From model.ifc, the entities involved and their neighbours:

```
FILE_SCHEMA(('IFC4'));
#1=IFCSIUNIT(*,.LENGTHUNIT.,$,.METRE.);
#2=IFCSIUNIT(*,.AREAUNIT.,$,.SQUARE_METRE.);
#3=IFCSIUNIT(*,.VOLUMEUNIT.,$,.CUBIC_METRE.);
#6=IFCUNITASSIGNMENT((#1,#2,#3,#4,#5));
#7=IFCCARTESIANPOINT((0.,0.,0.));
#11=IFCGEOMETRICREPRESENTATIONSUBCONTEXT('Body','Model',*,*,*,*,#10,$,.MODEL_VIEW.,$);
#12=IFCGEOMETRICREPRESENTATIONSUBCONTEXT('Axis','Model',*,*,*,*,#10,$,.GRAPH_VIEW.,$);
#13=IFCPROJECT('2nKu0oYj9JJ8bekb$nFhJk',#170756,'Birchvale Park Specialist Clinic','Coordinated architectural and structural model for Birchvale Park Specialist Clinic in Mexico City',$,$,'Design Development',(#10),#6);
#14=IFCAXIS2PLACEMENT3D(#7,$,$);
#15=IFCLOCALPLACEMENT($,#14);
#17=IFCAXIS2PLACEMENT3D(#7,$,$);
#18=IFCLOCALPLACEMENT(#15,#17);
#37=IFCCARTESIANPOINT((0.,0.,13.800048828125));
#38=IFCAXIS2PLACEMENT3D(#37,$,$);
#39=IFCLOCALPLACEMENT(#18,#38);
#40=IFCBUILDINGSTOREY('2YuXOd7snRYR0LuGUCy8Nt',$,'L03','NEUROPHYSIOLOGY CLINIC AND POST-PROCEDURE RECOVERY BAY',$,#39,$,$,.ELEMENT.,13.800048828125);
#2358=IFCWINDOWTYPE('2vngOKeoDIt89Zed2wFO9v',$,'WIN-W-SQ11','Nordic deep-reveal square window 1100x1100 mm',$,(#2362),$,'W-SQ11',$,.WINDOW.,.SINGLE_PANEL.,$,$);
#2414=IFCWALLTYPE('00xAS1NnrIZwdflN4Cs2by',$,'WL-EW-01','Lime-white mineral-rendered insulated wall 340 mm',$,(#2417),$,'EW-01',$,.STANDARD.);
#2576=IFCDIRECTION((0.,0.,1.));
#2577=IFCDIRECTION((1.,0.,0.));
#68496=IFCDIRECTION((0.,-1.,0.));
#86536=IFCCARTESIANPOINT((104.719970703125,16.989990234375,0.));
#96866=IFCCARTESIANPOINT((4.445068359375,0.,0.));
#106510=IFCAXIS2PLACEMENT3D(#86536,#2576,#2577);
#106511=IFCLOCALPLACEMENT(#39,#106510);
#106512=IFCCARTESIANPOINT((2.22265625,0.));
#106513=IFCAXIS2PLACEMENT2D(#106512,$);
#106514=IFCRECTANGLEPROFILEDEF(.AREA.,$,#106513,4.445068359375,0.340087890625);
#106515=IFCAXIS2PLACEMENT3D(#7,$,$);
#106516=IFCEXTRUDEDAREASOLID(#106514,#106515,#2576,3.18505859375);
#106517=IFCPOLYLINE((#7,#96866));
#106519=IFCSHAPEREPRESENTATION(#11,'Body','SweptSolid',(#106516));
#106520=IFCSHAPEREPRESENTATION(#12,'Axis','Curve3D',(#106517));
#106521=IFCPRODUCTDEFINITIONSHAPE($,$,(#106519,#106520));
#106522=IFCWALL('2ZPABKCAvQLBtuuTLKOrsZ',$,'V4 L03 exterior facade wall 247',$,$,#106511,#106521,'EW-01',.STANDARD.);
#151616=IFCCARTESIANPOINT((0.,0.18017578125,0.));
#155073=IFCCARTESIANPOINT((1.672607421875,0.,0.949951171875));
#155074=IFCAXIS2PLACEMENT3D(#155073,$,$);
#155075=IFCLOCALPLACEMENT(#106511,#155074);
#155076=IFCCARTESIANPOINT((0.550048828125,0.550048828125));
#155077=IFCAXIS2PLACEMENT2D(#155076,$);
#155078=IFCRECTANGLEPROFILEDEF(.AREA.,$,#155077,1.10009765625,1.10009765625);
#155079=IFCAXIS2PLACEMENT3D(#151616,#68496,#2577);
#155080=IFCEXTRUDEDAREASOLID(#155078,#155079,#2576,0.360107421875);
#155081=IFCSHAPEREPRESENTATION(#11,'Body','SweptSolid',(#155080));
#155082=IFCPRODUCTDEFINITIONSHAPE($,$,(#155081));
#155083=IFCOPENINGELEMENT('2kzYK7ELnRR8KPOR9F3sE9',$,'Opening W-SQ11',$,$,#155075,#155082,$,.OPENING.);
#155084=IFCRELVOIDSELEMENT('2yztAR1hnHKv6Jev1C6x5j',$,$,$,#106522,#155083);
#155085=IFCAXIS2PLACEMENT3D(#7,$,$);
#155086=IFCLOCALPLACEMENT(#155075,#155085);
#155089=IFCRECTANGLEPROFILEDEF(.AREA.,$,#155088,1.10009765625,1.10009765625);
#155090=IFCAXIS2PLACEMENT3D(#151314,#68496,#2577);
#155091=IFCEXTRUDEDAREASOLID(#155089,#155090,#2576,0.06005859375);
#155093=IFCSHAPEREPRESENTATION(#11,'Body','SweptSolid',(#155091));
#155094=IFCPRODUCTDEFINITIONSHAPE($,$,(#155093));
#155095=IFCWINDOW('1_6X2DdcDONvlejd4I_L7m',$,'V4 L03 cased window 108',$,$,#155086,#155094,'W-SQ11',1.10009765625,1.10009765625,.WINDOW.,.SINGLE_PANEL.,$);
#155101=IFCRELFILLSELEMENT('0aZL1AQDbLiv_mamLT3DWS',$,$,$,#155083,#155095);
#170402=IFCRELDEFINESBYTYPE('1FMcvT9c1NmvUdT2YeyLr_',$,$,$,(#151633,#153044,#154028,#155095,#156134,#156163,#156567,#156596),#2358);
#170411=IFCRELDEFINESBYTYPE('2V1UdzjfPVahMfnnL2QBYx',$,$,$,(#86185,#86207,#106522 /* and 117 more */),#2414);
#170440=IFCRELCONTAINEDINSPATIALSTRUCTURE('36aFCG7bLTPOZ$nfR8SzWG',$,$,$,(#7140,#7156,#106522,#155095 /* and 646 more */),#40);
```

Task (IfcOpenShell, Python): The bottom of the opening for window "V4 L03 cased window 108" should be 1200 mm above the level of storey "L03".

```python
import numpy as np
import ifcopenshell
import ifcopenshell.api.geometry
import ifcopenshell.geom
import ifcopenshell.util.element
import ifcopenshell.util.placement
import ifcopenshell.util.shape
import ifcopenshell.util.unit

model = ifcopenshell.open("model.ifc")
unit_scale = ifcopenshell.util.unit.calculate_unit_scale(model)

window = model.by_guid("1_6X2DdcDONvlejd4I_L7m")
opening = window.FillsVoids[0].RelatingOpeningElement
storey = ifcopenshell.util.element.get_container(window, ifc_class="IfcBuildingStorey")
level = ifcopenshell.util.placement.get_local_placement(storey.ObjectPlacement)[2, 3]

# The opening's origin need not be at the sill, so measure its lowest point.
shape = ifcopenshell.geom.create_shape(ifcopenshell.geom.settings(), opening)
bottom = ifcopenshell.util.shape.get_shape_bottom_elevation(shape, shape.geometry) / unit_scale
dz = level + 1.2 / unit_scale - bottom

shift = np.array([0.0, 0.0, dz])
# The window is placed relative to its opening, so it follows when the opening moves.
matrix = ifcopenshell.util.placement.get_local_placement(opening.ObjectPlacement)
matrix[:3, 3] += shift
ifcopenshell.api.geometry.edit_object_placement(
    model, product=opening, matrix=matrix, is_si=False, should_transform_children=True
)

print(f"moved by {dz * unit_scale:+.3f} m")

model.write("model_v2.ifc")
```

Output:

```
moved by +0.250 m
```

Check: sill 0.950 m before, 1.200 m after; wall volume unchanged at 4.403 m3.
